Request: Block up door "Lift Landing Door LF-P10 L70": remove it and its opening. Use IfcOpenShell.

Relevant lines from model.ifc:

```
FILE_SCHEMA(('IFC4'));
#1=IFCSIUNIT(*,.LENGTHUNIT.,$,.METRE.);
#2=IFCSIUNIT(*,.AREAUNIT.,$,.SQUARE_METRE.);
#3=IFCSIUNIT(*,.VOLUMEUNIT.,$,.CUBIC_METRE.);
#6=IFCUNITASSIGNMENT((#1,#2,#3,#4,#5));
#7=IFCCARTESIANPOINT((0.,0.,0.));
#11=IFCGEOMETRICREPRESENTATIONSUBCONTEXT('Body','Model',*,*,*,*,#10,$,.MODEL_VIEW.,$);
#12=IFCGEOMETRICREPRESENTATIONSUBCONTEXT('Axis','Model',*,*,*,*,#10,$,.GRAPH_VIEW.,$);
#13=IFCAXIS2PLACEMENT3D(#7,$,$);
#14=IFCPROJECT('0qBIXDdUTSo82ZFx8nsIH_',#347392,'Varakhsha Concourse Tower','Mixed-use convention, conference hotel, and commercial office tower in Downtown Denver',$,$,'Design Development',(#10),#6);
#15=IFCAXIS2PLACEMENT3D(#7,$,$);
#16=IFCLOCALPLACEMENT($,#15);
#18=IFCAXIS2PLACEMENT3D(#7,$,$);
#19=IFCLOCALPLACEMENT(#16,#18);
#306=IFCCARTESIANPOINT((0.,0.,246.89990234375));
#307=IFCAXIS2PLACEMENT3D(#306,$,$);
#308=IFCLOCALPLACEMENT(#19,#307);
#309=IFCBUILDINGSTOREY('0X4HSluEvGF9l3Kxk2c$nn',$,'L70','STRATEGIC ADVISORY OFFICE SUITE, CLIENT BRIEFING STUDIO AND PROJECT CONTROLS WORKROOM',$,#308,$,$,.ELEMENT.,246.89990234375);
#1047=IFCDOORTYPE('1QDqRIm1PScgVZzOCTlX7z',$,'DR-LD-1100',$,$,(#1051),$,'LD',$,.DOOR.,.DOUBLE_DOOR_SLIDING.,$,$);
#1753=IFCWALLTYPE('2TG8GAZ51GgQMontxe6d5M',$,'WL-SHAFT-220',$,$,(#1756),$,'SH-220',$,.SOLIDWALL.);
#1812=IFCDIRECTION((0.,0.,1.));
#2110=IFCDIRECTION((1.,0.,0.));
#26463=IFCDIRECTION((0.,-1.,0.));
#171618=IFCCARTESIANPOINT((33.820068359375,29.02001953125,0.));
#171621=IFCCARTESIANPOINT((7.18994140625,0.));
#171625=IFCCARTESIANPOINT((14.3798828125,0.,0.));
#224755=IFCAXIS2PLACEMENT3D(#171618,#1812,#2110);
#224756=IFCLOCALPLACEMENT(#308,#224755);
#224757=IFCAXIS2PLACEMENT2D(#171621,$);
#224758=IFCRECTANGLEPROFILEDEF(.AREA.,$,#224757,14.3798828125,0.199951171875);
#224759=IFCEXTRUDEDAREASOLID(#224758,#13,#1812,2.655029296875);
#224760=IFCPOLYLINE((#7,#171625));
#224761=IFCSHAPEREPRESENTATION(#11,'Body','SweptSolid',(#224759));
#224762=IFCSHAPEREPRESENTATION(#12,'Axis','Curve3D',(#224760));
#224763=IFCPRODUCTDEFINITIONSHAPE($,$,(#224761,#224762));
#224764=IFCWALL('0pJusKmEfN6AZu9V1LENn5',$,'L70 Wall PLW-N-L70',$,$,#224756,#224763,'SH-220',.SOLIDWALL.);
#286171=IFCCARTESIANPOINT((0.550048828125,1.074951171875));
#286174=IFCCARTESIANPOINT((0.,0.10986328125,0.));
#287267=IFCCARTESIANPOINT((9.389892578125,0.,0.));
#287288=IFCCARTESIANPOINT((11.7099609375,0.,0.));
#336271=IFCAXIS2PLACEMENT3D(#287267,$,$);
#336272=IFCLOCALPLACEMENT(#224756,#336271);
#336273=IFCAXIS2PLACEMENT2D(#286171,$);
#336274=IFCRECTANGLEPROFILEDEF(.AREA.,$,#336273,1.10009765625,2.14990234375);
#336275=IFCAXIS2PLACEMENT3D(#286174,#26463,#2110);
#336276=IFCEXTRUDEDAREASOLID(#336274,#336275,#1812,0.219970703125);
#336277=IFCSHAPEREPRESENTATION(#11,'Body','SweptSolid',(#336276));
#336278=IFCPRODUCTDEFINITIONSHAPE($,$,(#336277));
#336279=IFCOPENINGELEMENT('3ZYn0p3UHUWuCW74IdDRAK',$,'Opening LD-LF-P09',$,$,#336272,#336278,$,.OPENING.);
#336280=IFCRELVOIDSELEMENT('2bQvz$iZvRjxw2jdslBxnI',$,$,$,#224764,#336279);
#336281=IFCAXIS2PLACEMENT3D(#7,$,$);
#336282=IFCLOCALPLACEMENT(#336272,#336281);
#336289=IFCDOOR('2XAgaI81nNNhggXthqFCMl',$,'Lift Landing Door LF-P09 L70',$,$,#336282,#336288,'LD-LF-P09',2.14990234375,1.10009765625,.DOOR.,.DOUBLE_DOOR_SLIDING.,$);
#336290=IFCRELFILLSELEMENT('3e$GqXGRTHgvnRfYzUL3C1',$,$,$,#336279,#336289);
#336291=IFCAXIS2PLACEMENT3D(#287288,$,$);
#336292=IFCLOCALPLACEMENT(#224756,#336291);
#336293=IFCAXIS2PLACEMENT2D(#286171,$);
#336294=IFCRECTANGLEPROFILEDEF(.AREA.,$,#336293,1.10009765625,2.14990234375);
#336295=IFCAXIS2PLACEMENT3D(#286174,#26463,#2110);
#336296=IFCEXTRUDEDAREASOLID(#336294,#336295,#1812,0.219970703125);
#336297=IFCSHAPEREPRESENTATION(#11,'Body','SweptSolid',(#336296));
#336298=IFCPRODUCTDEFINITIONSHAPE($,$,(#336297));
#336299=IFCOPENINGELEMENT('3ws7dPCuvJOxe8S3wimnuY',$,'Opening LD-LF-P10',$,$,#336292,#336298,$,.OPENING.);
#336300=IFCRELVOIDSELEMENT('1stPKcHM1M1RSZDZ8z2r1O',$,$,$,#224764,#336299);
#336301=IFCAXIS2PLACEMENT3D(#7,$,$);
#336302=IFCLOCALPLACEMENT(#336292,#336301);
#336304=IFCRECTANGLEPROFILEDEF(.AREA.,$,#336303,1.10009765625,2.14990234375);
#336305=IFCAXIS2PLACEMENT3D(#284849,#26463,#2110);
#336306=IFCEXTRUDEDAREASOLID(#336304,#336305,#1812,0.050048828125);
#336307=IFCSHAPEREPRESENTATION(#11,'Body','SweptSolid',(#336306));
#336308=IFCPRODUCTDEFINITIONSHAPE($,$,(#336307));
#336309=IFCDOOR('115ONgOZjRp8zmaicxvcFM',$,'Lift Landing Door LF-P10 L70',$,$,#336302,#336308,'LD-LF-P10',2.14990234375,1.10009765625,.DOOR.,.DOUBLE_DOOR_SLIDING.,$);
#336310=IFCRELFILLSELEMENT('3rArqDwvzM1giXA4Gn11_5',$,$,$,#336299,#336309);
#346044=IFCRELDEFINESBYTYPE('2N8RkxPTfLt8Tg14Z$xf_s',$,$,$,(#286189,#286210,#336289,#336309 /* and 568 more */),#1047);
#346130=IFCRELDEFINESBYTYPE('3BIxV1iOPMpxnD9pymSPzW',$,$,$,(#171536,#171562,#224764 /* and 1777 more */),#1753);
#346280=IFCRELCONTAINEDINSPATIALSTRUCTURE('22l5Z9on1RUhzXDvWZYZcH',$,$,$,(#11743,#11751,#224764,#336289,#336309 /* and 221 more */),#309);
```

```python
import ifcopenshell
import ifcopenshell.api.feature
import ifcopenshell.api.root
import ifcopenshell.geom
import ifcopenshell.util.shape

model = ifcopenshell.open("model.ifc")
settings = ifcopenshell.geom.settings()


def volume(element):
    """Net volume in cubic metres, openings subtracted."""
    shape = ifcopenshell.geom.create_shape(settings, element)
    return ifcopenshell.util.shape.get_volume(shape.geometry)


door = model.by_guid("115ONgOZjRp8zmaicxvcFM")
opening = door.FillsVoids[0].RelatingOpeningElement
wall = opening.VoidsElements[0].RelatingBuildingElement
before = volume(wall)

ifcopenshell.api.root.remove_product(model, product=door)
ifcopenshell.api.feature.remove_feature(model, feature=opening)

after = volume(wall)

print(f"wall volume {before:.3f} -> {after:.3f} m3")

model.write("model-out.ifc")
```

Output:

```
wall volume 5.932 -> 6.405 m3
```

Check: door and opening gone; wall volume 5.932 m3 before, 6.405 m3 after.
